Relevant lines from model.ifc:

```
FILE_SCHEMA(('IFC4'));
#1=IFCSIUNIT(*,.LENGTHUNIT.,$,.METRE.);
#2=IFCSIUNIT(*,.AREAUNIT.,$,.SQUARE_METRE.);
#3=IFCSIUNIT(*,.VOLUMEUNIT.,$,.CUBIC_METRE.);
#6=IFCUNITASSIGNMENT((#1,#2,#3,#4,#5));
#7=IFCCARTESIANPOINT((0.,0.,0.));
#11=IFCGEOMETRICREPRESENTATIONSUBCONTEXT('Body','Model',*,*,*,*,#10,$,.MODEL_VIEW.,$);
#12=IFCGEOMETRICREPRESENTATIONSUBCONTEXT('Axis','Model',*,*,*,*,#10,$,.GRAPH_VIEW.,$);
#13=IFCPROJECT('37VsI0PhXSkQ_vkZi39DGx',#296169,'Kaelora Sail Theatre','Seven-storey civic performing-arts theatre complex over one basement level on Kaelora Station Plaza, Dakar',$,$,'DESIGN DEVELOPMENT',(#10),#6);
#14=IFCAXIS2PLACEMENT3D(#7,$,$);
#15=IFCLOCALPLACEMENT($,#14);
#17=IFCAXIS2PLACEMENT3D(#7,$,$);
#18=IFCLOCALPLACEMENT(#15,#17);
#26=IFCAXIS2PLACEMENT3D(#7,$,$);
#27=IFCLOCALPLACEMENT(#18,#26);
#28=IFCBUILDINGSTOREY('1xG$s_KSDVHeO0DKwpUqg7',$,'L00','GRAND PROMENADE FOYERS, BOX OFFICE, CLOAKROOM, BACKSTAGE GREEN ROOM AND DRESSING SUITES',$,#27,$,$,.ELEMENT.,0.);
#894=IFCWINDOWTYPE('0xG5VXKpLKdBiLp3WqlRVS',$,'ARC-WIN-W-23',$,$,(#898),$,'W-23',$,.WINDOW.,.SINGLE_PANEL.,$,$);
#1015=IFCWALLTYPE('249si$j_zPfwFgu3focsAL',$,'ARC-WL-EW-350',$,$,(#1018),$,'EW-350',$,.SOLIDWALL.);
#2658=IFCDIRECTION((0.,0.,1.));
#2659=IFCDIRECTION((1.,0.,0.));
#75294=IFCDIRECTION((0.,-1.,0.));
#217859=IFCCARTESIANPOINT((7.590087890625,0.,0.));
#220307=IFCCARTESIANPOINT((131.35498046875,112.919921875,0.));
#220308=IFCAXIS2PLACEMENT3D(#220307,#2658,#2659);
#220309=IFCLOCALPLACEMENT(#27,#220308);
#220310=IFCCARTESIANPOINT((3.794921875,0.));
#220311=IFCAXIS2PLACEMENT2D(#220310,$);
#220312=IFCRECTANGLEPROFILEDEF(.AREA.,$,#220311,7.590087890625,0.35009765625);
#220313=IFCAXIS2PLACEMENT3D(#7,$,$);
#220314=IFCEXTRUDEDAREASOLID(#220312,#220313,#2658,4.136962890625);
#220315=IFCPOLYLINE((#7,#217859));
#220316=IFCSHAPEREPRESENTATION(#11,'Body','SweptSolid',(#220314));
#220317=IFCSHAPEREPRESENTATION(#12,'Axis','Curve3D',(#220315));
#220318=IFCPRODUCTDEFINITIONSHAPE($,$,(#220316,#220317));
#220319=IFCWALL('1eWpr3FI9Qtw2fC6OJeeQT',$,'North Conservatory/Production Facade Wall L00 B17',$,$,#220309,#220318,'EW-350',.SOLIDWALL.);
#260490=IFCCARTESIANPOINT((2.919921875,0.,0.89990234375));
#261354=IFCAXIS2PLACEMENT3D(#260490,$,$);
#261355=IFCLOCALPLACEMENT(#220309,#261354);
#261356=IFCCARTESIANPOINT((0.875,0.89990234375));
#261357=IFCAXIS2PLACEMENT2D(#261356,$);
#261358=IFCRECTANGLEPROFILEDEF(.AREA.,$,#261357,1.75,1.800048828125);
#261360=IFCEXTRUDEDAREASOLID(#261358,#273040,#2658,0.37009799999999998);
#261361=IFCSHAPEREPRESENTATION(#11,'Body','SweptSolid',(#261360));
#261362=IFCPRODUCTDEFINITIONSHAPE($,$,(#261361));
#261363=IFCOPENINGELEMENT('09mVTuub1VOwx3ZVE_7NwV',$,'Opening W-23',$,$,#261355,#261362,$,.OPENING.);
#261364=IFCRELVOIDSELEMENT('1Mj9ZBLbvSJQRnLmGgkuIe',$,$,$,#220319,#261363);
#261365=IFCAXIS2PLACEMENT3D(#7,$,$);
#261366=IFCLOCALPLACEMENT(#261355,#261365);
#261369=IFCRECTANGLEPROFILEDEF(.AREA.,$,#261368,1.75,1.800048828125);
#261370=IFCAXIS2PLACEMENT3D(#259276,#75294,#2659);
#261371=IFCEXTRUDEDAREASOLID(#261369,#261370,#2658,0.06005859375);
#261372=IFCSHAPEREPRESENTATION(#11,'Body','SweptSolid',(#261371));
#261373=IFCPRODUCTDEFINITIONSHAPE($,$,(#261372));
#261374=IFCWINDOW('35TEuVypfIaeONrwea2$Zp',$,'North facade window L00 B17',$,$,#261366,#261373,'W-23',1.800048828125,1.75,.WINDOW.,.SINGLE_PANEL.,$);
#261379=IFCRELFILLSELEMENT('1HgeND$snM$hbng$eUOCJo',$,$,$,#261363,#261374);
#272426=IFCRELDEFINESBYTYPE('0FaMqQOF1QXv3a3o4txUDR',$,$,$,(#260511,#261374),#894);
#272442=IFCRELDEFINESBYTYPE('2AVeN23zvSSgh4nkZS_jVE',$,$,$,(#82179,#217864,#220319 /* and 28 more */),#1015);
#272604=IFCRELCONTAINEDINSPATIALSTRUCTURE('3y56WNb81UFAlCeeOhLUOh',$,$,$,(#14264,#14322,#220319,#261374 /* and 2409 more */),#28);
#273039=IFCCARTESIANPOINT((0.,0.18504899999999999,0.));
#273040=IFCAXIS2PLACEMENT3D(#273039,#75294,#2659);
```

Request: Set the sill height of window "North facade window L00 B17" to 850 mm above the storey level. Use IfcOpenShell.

```python
import numpy as np
import ifcopenshell
import ifcopenshell.api.geometry
import ifcopenshell.geom
import ifcopenshell.util.element
import ifcopenshell.util.placement
import ifcopenshell.util.shape
import ifcopenshell.util.unit

model = ifcopenshell.open("model.ifc")
unit_scale = ifcopenshell.util.unit.calculate_unit_scale(model)

window = model.by_guid("35TEuVypfIaeONrwea2$Zp")
opening = window.FillsVoids[0].RelatingOpeningElement
storey = ifcopenshell.util.element.get_container(window, ifc_class="IfcBuildingStorey")
level = ifcopenshell.util.placement.get_local_placement(storey.ObjectPlacement)[2, 3]

# The opening's origin need not be at the sill, so measure its lowest point.
shape = ifcopenshell.geom.create_shape(ifcopenshell.geom.settings(), opening)
bottom = ifcopenshell.util.shape.get_shape_bottom_elevation(shape, shape.geometry) / unit_scale
dz = level + 0.85 / unit_scale - bottom

shift = np.array([0.0, 0.0, dz])
# The window is placed relative to its opening, so it follows when the opening moves.
matrix = ifcopenshell.util.placement.get_local_placement(opening.ObjectPlacement)
matrix[:3, 3] += shift
ifcopenshell.api.geometry.edit_object_placement(
    model, product=opening, matrix=matrix, is_si=False, should_transform_children=True
)

print(f"moved by {dz * unit_scale:+.3f} m")

model.write("model_rev.ifc")
```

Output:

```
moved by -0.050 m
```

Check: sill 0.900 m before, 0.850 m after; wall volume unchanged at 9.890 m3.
